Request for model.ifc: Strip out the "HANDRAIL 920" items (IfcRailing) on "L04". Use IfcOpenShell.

First a look at what the model holds.

```python
import ifcopenshell
import ifcopenshell.util.element

model = ifcopenshell.open("model.ifc")
print(model.schema)
storey = next(s for s in model.by_type("IfcBuildingStorey") if s.Name == "L04")
railings = [e for e in ifcopenshell.util.element.get_decomposition(storey) if e.is_a("IfcRailing")]
seen = {}
for e in railings:
    element_type = ifcopenshell.util.element.get_type(e)
    name = element_type.Name if element_type not in (None, e) else None
    seen[name] = seen.get(name, 0) + 1
for name, count in sorted(seen.items(), key=str):
    print(count, "x", name)
```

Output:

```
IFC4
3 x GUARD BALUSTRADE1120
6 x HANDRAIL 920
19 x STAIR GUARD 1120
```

```python
import ifcopenshell
import ifcopenshell.api.root
import ifcopenshell.util.element

model = ifcopenshell.open("model.ifc")

storey = next(s for s in model.by_type("IfcBuildingStorey") if s.Name == "L04")
railings = [e for e in ifcopenshell.util.element.get_decomposition(storey) if e.is_a("IfcRailing")]
targets = [e for e in railings if (t := ifcopenshell.util.element.get_type(e)) not in (None, e) and t.Name == "HANDRAIL 920"]

for e in targets:
    ifcopenshell.api.root.remove_product(model, product=e)
print(len(targets), "removed")

model.write("model_v2.ifc")
```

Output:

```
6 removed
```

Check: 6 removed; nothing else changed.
